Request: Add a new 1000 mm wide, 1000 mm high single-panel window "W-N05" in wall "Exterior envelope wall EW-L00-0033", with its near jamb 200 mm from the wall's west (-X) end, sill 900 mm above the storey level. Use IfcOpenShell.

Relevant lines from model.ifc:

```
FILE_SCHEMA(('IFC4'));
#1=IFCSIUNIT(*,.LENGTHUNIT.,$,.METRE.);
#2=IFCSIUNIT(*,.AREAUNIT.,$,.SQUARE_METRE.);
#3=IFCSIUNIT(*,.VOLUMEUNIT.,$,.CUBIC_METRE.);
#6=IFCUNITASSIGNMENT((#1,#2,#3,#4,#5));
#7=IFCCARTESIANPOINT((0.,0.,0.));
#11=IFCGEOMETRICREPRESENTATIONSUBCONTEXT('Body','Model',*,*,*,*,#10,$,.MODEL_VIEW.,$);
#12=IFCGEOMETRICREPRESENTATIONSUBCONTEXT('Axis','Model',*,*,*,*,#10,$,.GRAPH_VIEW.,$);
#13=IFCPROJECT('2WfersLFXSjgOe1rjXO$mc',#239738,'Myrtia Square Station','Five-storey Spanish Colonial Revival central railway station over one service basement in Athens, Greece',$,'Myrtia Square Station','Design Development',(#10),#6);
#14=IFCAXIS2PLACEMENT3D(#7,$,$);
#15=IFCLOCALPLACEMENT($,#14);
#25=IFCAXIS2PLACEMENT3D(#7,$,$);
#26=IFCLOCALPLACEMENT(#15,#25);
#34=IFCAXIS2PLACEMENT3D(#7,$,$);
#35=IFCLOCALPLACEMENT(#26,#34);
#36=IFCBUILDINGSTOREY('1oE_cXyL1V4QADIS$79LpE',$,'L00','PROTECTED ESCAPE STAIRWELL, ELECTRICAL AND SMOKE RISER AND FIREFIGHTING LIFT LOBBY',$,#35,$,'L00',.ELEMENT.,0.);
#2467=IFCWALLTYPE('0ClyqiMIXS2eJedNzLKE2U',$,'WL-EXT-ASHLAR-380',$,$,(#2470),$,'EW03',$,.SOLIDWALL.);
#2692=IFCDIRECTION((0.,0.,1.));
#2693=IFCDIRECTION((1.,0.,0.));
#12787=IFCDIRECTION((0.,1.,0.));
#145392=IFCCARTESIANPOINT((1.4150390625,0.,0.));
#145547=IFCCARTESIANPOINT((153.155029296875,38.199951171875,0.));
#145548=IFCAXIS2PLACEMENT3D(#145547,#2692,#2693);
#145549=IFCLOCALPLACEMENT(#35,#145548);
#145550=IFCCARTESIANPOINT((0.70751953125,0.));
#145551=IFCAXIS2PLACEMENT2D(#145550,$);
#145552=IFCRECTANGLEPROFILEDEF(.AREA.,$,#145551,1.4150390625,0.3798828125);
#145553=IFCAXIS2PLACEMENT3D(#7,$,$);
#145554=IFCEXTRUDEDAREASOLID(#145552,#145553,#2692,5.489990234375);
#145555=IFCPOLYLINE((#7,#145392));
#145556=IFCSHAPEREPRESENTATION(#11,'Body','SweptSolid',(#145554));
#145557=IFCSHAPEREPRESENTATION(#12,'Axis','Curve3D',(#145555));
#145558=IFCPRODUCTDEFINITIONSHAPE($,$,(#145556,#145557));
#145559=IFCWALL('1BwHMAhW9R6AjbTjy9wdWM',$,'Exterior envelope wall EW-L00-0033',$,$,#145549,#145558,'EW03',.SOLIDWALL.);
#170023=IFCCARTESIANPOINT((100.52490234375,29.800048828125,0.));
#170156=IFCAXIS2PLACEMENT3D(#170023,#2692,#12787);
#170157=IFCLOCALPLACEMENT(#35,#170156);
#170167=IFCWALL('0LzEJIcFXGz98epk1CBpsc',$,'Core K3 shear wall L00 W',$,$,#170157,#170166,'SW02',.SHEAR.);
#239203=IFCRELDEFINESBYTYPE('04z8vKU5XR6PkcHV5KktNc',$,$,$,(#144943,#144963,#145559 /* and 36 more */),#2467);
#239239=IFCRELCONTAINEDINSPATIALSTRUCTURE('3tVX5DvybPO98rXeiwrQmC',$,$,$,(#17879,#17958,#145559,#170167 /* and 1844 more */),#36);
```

```python
import numpy as np
import ifcopenshell
import ifcopenshell.api.feature
import ifcopenshell.api.geometry
import ifcopenshell.api.root
import ifcopenshell.api.spatial
import ifcopenshell.geom
import ifcopenshell.util.element
import ifcopenshell.util.placement
import ifcopenshell.util.representation
import ifcopenshell.util.shape
import ifcopenshell.util.unit

model = ifcopenshell.open("model.ifc")
unit_scale = ifcopenshell.util.unit.calculate_unit_scale(model)
settings = ifcopenshell.geom.settings()


def volume(element):
    """Net volume in cubic metres, openings subtracted."""
    shape = ifcopenshell.geom.create_shape(settings, element)
    return ifcopenshell.util.shape.get_volume(shape.geometry)


wall = model.by_id(145559)
storey = ifcopenshell.util.element.get_container(wall, ifc_class="IfcBuildingStorey")
context = ifcopenshell.util.representation.get_context(model, "Model", "Body", "MODEL_VIEW")
before = volume(wall)

width, height, from_end, sill = 1, 1, 0.2, 0.9  # metres

# The wall runs along its own X axis, and the end named is its -X end.
wall_shape = ifcopenshell.geom.create_shape(settings, wall)
x, y, z = ifcopenshell.util.shape.get_vertices(wall_shape.geometry).T
start = x.min() + from_end
face, thickness = float(y.min()), float(y.max() - y.min())
wall_matrix = ifcopenshell.util.placement.get_local_placement(wall.ObjectPlacement)
level = ifcopenshell.util.placement.get_local_placement(storey.ObjectPlacement)[2, 3]


def in_wall(x, y):
    """Placement at x, y metres in the wall's axes, at sill height."""
    matrix = wall_matrix.copy()
    matrix[:, 3] = wall_matrix @ np.array([x / unit_scale, y / unit_scale, 0.0, 1.0])
    matrix[2, 3] = level + sill / unit_scale
    return matrix


# Opening: a box that overshoots both wall faces by 50 mm.
opening = ifcopenshell.api.root.create_entity(model, ifc_class="IfcOpeningElement", predefined_type="OPENING")
box = ifcopenshell.api.geometry.add_wall_representation(
    model, context=context, length=width, height=height, thickness=thickness + 0.1
)
ifcopenshell.api.geometry.assign_representation(model, product=opening, representation=box)
ifcopenshell.api.geometry.edit_object_placement(model, product=opening, matrix=in_wall(start, face - 0.05), is_si=False)
ifcopenshell.api.feature.add_feature(model, feature=opening, element=wall)

window = ifcopenshell.api.root.create_entity(model, ifc_class="IfcWindow", name="W-N05", predefined_type="WINDOW")
window.OverallWidth, window.OverallHeight = width / unit_scale, height / unit_scale
window.PartitioningType = "SINGLE_PANEL"
body = ifcopenshell.api.geometry.add_window_representation(
    model,
    context=context,
    overall_width=window.OverallWidth,
    overall_height=window.OverallHeight,
    partition_type="SINGLE_PANEL",
)
ifcopenshell.api.geometry.assign_representation(model, product=window, representation=body)
ifcopenshell.api.spatial.assign_container(model, products=[window], relating_structure=storey)
ifcopenshell.api.feature.add_filling(model, opening=opening, element=window)

# Centre the window in the wall's thickness.
ifcopenshell.api.geometry.edit_object_placement(model, product=window, matrix=in_wall(start, face), is_si=False)
window_shape = ifcopenshell.geom.create_shape(settings, window)
depth = ifcopenshell.util.shape.get_vertices(window_shape.geometry)[:, 1]
offset = face + thickness / 2 - (depth.min() + depth.max()) / 2
ifcopenshell.api.geometry.edit_object_placement(model, product=window, matrix=in_wall(start, offset), is_si=False)

after = volume(wall)

print(f"wall volume {before:.3f} -> {after:.3f} m3")

model.write("model_v2.ifc")
```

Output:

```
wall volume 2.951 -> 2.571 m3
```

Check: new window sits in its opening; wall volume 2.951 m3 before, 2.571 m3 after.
